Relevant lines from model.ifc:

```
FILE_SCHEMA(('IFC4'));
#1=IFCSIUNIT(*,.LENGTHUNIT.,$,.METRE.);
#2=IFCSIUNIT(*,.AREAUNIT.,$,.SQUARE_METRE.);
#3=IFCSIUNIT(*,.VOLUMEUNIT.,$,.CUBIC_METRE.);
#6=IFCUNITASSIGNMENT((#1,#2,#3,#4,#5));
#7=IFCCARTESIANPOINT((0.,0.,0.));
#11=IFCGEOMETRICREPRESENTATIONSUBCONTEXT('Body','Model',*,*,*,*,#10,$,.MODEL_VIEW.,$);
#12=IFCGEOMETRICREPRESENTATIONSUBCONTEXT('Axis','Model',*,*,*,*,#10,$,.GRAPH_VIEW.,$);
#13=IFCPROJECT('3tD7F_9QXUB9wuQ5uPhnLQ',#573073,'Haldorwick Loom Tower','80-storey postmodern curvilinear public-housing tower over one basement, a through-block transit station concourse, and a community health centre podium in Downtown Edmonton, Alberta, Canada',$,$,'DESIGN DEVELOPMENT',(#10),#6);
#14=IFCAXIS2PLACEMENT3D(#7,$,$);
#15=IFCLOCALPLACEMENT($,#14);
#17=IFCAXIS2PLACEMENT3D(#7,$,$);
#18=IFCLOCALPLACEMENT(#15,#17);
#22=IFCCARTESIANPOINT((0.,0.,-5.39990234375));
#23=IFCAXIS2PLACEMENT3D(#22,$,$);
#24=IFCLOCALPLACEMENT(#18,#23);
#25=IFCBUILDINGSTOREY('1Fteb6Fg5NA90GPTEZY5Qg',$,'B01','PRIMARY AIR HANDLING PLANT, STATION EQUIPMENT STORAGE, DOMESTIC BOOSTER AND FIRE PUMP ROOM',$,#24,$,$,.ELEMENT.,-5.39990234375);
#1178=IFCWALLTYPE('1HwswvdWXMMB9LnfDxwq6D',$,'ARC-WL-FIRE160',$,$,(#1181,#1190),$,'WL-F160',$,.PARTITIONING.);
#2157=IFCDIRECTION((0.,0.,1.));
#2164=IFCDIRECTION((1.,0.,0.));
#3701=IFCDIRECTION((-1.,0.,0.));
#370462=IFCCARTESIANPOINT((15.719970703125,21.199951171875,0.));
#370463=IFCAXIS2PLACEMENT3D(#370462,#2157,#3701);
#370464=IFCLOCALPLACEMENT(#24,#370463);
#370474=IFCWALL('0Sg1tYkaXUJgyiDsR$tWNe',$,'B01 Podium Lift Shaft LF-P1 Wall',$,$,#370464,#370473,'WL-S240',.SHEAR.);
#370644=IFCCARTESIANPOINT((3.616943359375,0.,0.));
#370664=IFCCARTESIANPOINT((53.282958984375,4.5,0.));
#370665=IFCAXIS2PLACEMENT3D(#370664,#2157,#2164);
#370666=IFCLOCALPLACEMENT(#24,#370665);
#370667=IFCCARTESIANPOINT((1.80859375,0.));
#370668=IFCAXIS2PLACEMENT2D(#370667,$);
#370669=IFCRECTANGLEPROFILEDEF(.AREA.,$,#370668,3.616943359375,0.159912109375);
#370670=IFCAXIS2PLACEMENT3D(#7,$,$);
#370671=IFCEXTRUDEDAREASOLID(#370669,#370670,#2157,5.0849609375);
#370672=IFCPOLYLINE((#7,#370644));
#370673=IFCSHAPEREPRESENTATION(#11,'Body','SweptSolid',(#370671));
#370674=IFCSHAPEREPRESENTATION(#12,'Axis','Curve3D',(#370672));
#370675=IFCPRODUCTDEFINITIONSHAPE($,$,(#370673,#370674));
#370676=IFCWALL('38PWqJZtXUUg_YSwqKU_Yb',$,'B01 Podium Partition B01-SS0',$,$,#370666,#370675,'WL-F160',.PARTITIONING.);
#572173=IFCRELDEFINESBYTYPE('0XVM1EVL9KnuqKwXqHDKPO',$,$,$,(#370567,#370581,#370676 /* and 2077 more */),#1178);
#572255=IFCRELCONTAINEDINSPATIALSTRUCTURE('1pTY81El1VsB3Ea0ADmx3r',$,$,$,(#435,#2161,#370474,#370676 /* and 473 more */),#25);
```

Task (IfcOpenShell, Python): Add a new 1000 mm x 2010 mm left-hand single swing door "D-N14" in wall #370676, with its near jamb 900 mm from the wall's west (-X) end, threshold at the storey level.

```python
import numpy as np
import ifcopenshell
import ifcopenshell.api.feature
import ifcopenshell.api.geometry
import ifcopenshell.api.root
import ifcopenshell.api.spatial
import ifcopenshell.geom
import ifcopenshell.util.element
import ifcopenshell.util.placement
import ifcopenshell.util.representation
import ifcopenshell.util.shape
import ifcopenshell.util.unit

model = ifcopenshell.open("model.ifc")
unit_scale = ifcopenshell.util.unit.calculate_unit_scale(model)
settings = ifcopenshell.geom.settings()


def volume(element):
    """Net volume in cubic metres, openings subtracted."""
    shape = ifcopenshell.geom.create_shape(settings, element)
    return ifcopenshell.util.shape.get_volume(shape.geometry)


wall = model.by_guid("38PWqJZtXUUg_YSwqKU_Yb")
storey = ifcopenshell.util.element.get_container(wall, ifc_class="IfcBuildingStorey")
context = ifcopenshell.util.representation.get_context(model, "Model", "Body", "MODEL_VIEW")
before = volume(wall)

width, height, from_end, sill = 1, 2.01, 0.9, 0.0  # metres

# The wall runs along its own X axis, and the end named is its -X end.
wall_shape = ifcopenshell.geom.create_shape(settings, wall)
x, y, z = ifcopenshell.util.shape.get_vertices(wall_shape.geometry).T
start = x.min() + from_end
face, thickness = float(y.min()), float(y.max() - y.min())
wall_matrix = ifcopenshell.util.placement.get_local_placement(wall.ObjectPlacement)
level = ifcopenshell.util.placement.get_local_placement(storey.ObjectPlacement)[2, 3]


def in_wall(x, y):
    """Placement at x, y metres in the wall's axes, at sill height."""
    matrix = wall_matrix.copy()
    matrix[:, 3] = wall_matrix @ np.array([x / unit_scale, y / unit_scale, 0.0, 1.0])
    matrix[2, 3] = level + sill / unit_scale
    return matrix


# Opening: a box that overshoots both wall faces by 50 mm.
opening = ifcopenshell.api.root.create_entity(model, ifc_class="IfcOpeningElement", predefined_type="OPENING")
box = ifcopenshell.api.geometry.add_wall_representation(
    model, context=context, length=width, height=height, thickness=thickness + 0.1
)
ifcopenshell.api.geometry.assign_representation(model, product=opening, representation=box)
ifcopenshell.api.geometry.edit_object_placement(model, product=opening, matrix=in_wall(start, face - 0.05), is_si=False)
ifcopenshell.api.feature.add_feature(model, feature=opening, element=wall)

door = ifcopenshell.api.root.create_entity(model, ifc_class="IfcDoor", name="D-N14", predefined_type="DOOR")
door.OverallWidth, door.OverallHeight = width / unit_scale, height / unit_scale
door.OperationType = "SINGLE_SWING_LEFT"
body = ifcopenshell.api.geometry.add_door_representation(
    model,
    context=context,
    overall_width=door.OverallWidth,
    overall_height=door.OverallHeight,
    operation_type="SINGLE_SWING_LEFT",
    lining_properties={"LiningDepth": thickness / unit_scale, "ThresholdDepth": thickness / unit_scale},
)
ifcopenshell.api.geometry.assign_representation(model, product=door, representation=body)
ifcopenshell.api.spatial.assign_container(model, products=[door], relating_structure=storey)
ifcopenshell.api.feature.add_filling(model, opening=opening, element=door)

# The lining spans the wall, so the door starts at the wall face.
ifcopenshell.api.geometry.edit_object_placement(model, product=door, matrix=in_wall(start, face), is_si=False)

after = volume(wall)

print(f"wall volume {before:.3f} -> {after:.3f} m3")

model.write("model_v2.ifc")
```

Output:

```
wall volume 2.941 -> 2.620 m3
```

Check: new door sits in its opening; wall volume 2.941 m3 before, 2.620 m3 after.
